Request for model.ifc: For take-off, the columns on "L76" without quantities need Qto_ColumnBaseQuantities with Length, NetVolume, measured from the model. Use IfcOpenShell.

First a look at what the model holds.

```python
import ifcopenshell
import ifcopenshell.util.element
import ifcopenshell.util.unit

model = ifcopenshell.open("model.ifc")
print(model.schema)
for unit_type in ("LENGTHUNIT", "AREAUNIT", "VOLUMEUNIT"):
    print(unit_type, ifcopenshell.util.unit.calculate_unit_scale(model, unit_type))
storey = next(s for s in model.by_type("IfcBuildingStorey") if s.Name == "L76")
columns = [e for e in ifcopenshell.util.element.get_decomposition(storey) if e.is_a("IfcColumn")]
for e in sorted(columns, key=lambda e: e.id()):
    print(e.id(), e.is_a(), e.Name, list(ifcopenshell.util.element.get_psets(e, qtos_only=True)), sep=" | ")
```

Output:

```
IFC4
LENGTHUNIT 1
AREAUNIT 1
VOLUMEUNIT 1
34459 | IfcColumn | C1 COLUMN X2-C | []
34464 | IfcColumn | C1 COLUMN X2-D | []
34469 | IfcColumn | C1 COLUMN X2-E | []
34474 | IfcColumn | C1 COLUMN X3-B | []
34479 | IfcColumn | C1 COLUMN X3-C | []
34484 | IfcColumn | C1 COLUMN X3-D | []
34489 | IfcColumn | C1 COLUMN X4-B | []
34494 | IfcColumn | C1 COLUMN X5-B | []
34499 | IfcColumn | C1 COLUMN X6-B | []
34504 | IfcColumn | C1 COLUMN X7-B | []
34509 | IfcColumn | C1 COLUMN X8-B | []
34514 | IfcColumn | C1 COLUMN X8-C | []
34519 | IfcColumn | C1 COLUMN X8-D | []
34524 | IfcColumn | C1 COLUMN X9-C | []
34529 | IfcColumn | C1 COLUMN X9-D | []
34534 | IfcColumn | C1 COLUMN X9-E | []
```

```python
import ifcopenshell
import ifcopenshell.api.pset
import ifcopenshell.geom
import ifcopenshell.util.element
import ifcopenshell.util.shape
import ifcopenshell.util.unit

model = ifcopenshell.open("model.ifc")
unit_scale = ifcopenshell.util.unit.calculate_unit_scale(model)
volume_scale = ifcopenshell.util.unit.calculate_unit_scale(model, "VOLUMEUNIT")
settings = ifcopenshell.geom.settings()

storey = next(s for s in model.by_type("IfcBuildingStorey") if s.Name == "L76")
columns = [e for e in ifcopenshell.util.element.get_decomposition(storey) if e.is_a("IfcColumn")]

for e in sorted(columns, key=lambda e: e.id()):
    if ifcopenshell.util.element.get_psets(e, qtos_only=True, should_inherit=False):
        continue
    # Geometry comes back in metres, in the element's own axes.
    shape = ifcopenshell.geom.create_shape(settings, e)
    values = {
        "Length": ifcopenshell.util.shape.get_z(shape.geometry) / unit_scale,
        "NetVolume": ifcopenshell.util.shape.get_volume(shape.geometry) / volume_scale,
    }
    qto = ifcopenshell.api.pset.add_qto(model, product=e, name="Qto_ColumnBaseQuantities")
    ifcopenshell.api.pset.edit_qto(model, qto=qto, properties=values)
    print(e.id(), {k: round(v, 3) for k, v in values.items()})

model.write("model_updated.ifc")
```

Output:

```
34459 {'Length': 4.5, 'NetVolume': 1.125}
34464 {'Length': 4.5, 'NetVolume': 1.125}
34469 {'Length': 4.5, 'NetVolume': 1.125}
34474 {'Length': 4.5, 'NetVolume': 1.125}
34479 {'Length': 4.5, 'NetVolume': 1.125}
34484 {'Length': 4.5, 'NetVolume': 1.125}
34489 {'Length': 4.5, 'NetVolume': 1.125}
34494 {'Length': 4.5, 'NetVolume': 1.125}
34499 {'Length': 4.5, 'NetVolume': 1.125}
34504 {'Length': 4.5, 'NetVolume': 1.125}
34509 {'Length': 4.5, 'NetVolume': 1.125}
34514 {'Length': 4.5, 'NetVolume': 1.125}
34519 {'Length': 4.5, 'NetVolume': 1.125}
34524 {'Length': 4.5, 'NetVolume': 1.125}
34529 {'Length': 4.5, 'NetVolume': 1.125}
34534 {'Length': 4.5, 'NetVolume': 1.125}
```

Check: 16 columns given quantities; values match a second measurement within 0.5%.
